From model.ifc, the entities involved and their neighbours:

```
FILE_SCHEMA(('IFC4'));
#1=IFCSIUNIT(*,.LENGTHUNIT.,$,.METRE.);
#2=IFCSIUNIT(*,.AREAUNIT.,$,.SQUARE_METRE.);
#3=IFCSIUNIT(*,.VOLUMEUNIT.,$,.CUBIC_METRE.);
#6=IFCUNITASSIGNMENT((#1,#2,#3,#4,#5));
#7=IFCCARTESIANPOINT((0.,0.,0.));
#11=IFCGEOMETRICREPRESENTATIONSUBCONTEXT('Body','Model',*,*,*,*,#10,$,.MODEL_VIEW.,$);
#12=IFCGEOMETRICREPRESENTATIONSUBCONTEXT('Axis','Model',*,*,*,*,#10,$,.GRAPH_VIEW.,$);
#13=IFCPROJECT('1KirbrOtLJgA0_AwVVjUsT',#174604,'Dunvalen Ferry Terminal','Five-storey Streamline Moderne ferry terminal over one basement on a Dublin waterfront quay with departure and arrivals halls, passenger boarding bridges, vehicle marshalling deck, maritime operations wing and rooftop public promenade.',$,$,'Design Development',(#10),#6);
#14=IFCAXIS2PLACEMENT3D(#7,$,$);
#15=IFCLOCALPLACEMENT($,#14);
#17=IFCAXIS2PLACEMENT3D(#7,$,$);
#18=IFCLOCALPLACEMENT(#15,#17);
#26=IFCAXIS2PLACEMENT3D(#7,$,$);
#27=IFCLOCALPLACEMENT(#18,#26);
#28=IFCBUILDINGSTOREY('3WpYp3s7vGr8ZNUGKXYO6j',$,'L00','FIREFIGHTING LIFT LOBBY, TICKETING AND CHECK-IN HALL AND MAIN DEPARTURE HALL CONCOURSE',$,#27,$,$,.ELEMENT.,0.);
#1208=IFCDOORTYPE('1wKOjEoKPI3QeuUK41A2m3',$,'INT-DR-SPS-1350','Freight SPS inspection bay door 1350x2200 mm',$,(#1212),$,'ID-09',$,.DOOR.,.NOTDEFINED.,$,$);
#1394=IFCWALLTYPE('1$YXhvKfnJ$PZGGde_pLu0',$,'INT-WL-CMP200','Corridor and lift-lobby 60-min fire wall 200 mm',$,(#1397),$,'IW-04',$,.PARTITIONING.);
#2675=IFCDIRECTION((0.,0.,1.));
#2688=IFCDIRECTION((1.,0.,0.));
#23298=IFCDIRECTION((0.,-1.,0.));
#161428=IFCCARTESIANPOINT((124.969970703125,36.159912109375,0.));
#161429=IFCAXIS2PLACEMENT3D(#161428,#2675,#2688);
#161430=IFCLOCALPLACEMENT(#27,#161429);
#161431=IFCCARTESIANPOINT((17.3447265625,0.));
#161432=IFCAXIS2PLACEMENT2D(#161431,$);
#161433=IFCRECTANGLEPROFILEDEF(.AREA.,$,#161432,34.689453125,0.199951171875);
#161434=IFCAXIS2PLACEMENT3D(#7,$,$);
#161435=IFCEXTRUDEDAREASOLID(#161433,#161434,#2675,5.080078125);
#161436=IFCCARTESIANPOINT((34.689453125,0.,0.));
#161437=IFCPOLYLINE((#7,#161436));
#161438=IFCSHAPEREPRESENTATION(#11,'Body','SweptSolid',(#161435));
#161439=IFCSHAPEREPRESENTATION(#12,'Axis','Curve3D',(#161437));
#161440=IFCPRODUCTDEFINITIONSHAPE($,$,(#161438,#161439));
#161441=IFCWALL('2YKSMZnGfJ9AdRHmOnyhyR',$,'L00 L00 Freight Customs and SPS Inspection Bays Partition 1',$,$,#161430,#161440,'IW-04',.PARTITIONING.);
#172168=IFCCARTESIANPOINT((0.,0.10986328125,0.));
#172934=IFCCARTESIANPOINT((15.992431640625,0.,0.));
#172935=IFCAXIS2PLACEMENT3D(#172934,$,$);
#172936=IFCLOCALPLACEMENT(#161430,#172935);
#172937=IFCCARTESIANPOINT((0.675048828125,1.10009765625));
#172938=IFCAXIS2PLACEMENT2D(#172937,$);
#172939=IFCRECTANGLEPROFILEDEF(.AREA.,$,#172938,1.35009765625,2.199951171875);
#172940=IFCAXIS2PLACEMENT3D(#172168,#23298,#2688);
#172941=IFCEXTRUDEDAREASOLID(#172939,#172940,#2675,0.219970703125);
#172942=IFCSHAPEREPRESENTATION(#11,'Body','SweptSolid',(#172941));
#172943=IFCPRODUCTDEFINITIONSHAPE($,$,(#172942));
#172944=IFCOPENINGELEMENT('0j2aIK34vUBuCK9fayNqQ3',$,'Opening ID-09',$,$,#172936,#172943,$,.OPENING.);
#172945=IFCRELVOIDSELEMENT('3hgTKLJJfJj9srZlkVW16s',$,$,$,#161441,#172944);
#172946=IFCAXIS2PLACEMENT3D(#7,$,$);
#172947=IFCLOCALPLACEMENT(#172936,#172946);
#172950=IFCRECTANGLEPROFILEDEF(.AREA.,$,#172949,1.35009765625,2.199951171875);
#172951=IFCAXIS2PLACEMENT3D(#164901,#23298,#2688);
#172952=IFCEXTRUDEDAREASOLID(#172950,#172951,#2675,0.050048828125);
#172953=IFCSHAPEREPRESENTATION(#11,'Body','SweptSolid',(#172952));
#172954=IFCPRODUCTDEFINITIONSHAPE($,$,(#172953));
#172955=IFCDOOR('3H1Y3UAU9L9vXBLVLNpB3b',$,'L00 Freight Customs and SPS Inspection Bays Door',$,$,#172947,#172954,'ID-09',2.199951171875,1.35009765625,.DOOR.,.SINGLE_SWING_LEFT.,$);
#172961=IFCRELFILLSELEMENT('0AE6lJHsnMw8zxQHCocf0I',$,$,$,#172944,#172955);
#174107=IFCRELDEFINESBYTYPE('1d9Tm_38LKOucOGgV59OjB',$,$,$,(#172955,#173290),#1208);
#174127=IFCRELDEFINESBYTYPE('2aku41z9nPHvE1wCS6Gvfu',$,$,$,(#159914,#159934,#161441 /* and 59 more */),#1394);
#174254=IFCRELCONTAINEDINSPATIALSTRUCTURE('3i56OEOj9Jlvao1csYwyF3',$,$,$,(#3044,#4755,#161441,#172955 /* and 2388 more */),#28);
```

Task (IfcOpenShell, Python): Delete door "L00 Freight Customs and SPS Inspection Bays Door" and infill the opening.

```python
import ifcopenshell
import ifcopenshell.api.feature
import ifcopenshell.api.root
import ifcopenshell.geom
import ifcopenshell.util.shape

model = ifcopenshell.open("model.ifc")
settings = ifcopenshell.geom.settings()


def volume(element):
    """Net volume in cubic metres, openings subtracted."""
    shape = ifcopenshell.geom.create_shape(settings, element)
    return ifcopenshell.util.shape.get_volume(shape.geometry)


door = model.by_guid("3H1Y3UAU9L9vXBLVLNpB3b")
opening = door.FillsVoids[0].RelatingOpeningElement
wall = opening.VoidsElements[0].RelatingBuildingElement
before = volume(wall)

ifcopenshell.api.root.remove_product(model, product=door)
ifcopenshell.api.feature.remove_feature(model, feature=opening)

after = volume(wall)

print(f"wall volume {before:.3f} -> {after:.3f} m3")

model.write("model_edited.ifc")
```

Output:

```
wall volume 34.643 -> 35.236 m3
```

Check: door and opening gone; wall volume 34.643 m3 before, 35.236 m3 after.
